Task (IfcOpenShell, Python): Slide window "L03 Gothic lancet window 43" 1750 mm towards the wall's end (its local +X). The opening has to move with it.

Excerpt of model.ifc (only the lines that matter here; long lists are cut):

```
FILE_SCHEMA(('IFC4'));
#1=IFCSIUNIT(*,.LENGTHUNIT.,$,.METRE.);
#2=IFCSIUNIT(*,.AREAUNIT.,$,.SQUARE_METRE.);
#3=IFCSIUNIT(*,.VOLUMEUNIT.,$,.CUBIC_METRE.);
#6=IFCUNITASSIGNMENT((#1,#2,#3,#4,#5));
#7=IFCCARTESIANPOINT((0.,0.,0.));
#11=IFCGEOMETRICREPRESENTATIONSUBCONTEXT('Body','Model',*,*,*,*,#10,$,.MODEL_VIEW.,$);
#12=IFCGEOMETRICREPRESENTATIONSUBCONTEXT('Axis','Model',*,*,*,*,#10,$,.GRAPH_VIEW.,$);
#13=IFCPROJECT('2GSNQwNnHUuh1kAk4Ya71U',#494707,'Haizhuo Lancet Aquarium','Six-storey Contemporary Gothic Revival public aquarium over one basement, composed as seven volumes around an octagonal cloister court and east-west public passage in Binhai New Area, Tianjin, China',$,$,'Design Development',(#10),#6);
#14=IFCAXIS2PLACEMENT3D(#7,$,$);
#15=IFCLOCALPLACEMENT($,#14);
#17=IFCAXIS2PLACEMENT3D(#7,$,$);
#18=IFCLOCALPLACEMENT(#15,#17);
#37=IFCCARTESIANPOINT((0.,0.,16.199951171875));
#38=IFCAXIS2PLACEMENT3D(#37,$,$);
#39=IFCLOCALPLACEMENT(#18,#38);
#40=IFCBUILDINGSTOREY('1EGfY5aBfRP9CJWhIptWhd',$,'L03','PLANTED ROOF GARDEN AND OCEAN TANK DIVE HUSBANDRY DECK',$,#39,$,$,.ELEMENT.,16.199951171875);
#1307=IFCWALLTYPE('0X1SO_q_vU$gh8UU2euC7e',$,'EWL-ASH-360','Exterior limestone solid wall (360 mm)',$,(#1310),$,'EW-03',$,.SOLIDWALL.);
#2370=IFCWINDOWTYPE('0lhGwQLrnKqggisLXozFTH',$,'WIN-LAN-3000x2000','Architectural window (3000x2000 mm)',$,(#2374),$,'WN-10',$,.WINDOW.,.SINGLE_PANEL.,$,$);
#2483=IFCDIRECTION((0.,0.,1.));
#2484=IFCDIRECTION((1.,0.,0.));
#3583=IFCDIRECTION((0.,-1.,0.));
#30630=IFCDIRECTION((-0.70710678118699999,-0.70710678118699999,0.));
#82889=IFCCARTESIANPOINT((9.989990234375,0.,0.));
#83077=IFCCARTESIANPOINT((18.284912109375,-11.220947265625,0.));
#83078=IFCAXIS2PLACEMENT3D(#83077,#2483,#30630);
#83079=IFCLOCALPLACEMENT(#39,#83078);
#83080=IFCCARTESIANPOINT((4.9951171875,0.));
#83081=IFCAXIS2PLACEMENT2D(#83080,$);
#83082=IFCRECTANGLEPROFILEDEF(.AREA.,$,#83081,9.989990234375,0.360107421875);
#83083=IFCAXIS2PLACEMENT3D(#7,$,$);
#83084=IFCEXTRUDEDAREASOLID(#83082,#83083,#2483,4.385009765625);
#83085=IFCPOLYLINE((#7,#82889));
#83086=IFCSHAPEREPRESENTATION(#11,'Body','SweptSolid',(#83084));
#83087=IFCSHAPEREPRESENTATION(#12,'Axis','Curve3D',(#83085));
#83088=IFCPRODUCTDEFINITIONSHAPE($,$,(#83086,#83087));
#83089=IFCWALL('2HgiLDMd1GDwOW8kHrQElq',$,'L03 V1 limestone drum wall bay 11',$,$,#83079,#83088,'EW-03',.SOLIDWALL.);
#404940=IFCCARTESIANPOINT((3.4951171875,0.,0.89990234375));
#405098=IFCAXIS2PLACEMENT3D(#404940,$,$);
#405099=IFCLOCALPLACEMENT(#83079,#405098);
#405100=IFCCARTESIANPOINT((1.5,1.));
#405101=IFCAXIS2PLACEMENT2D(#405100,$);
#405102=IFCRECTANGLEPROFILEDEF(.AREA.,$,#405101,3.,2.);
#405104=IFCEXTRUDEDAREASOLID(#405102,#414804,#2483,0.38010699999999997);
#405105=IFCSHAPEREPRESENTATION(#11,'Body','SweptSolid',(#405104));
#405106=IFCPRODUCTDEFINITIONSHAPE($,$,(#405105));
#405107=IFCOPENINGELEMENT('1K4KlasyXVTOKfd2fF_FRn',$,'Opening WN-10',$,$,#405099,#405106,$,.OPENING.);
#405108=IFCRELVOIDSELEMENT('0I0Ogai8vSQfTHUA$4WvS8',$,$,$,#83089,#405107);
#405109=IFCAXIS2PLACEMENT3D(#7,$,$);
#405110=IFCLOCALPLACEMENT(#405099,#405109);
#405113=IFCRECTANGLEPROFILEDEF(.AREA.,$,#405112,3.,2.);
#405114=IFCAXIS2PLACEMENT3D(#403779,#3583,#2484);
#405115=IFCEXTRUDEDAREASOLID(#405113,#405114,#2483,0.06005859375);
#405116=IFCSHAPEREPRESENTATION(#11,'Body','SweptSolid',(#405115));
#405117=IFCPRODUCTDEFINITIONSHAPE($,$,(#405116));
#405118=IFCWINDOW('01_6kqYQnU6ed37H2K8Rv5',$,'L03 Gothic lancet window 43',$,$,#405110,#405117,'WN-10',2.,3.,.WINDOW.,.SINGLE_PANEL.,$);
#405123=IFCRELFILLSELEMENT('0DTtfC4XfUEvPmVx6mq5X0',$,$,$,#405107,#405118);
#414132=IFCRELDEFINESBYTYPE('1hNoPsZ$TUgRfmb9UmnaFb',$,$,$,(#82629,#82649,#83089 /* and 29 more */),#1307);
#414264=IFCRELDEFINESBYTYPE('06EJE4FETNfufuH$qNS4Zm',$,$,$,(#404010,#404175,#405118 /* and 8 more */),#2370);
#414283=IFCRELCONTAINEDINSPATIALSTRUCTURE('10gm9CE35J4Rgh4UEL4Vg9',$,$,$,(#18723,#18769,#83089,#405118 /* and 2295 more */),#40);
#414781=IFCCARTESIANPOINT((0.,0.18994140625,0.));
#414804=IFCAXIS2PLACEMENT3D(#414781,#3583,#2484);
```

```python
import ifcopenshell
import ifcopenshell.api.geometry
import ifcopenshell.util.placement

model = ifcopenshell.open("model.ifc")

window = model.by_guid("01_6kqYQnU6ed37H2K8Rv5")
opening = window.FillsVoids[0].RelatingOpeningElement
wall = opening.VoidsElements[0].RelatingBuildingElement

wall_matrix = ifcopenshell.util.placement.get_local_placement(wall.ObjectPlacement)
shift = wall_matrix[:3, 0] * 1.75
before = ifcopenshell.util.placement.get_local_placement(window.ObjectPlacement)[:3, 3].copy()

# The window is placed relative to its opening, so it follows when the opening moves.
matrix = ifcopenshell.util.placement.get_local_placement(opening.ObjectPlacement)
matrix[:3, 3] += shift
ifcopenshell.api.geometry.edit_object_placement(
    model, product=opening, matrix=matrix, is_si=False, should_transform_children=True
)

after = ifcopenshell.util.placement.get_local_placement(window.ObjectPlacement)[:3, 3]
print("window moved by", (after - before).round(3) + 0.0)

model.write("model_updated.ifc")
```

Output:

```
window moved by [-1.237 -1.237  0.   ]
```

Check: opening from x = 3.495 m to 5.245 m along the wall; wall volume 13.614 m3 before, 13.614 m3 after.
